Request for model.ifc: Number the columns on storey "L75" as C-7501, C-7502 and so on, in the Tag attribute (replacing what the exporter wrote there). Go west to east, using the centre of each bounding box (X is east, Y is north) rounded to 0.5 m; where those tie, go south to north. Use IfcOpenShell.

First a look at what the model holds.

```python
import ifcopenshell
import ifcopenshell.util.element
import ifcopenshell.util.placement

model = ifcopenshell.open("model.ifc")
print(model.schema)
storey = next(s for s in model.by_type("IfcBuildingStorey") if s.Name == "L75")
columns = [e for e in ifcopenshell.util.element.get_decomposition(storey) if e.is_a("IfcColumn")]
for e in sorted(columns, key=lambda e: e.id()):
    origin = ifcopenshell.util.placement.get_local_placement(e.ObjectPlacement)[:3, 3]
    print(e.id(), e.Tag, e.Name, origin.round(2) + 0.0, sep=" | ")
```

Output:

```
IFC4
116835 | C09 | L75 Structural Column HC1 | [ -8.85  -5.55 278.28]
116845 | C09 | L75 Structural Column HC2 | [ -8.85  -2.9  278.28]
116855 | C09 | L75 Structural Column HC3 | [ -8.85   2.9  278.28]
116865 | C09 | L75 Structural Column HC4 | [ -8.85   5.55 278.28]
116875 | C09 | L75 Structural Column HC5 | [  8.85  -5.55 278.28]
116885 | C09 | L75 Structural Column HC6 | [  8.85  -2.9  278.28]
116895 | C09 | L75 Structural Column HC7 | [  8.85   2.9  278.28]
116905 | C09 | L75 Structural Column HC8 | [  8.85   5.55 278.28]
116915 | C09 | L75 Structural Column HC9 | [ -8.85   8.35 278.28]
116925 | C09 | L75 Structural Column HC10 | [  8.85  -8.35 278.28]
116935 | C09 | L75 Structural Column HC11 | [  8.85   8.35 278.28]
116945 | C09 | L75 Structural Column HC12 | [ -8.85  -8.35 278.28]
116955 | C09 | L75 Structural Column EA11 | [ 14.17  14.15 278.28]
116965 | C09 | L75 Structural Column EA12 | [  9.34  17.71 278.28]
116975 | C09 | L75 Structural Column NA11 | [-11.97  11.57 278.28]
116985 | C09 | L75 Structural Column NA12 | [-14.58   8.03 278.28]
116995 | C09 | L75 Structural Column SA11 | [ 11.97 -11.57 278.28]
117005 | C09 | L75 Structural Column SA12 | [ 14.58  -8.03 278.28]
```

```python
import ifcopenshell
import ifcopenshell.geom
import ifcopenshell.util.element
import ifcopenshell.util.shape

model = ifcopenshell.open("model.ifc")
settings = ifcopenshell.geom.settings()
settings.set("use-world-coords", True)


def centre(element):
    shape = ifcopenshell.geom.create_shape(settings, element)
    return ifcopenshell.util.shape.get_bbox_centroid(shape.geometry)


storey = next(s for s in model.by_type("IfcBuildingStorey") if s.Name == "L75")
columns = [e for e in ifcopenshell.util.element.get_decomposition(storey) if e.is_a("IfcColumn")]

# Insertion points can sit at a corner or the storey origin, so sort by the geometry (in metres).
centres = {e: centre(e) for e in columns}
columns.sort(key=lambda e: (round(centres[e][0] / 0.5), centres[e][1]))

for i, e in enumerate(columns, start=1):
    number = f"C-75{i:02d}"
    e.Tag = number
    print(e.id(), number)

model.write("model_updated.ifc")
```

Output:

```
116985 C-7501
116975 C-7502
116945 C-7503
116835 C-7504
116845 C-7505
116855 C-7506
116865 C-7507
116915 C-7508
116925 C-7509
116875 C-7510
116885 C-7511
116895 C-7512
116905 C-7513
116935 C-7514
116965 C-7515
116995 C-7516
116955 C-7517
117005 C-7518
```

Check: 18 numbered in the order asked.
